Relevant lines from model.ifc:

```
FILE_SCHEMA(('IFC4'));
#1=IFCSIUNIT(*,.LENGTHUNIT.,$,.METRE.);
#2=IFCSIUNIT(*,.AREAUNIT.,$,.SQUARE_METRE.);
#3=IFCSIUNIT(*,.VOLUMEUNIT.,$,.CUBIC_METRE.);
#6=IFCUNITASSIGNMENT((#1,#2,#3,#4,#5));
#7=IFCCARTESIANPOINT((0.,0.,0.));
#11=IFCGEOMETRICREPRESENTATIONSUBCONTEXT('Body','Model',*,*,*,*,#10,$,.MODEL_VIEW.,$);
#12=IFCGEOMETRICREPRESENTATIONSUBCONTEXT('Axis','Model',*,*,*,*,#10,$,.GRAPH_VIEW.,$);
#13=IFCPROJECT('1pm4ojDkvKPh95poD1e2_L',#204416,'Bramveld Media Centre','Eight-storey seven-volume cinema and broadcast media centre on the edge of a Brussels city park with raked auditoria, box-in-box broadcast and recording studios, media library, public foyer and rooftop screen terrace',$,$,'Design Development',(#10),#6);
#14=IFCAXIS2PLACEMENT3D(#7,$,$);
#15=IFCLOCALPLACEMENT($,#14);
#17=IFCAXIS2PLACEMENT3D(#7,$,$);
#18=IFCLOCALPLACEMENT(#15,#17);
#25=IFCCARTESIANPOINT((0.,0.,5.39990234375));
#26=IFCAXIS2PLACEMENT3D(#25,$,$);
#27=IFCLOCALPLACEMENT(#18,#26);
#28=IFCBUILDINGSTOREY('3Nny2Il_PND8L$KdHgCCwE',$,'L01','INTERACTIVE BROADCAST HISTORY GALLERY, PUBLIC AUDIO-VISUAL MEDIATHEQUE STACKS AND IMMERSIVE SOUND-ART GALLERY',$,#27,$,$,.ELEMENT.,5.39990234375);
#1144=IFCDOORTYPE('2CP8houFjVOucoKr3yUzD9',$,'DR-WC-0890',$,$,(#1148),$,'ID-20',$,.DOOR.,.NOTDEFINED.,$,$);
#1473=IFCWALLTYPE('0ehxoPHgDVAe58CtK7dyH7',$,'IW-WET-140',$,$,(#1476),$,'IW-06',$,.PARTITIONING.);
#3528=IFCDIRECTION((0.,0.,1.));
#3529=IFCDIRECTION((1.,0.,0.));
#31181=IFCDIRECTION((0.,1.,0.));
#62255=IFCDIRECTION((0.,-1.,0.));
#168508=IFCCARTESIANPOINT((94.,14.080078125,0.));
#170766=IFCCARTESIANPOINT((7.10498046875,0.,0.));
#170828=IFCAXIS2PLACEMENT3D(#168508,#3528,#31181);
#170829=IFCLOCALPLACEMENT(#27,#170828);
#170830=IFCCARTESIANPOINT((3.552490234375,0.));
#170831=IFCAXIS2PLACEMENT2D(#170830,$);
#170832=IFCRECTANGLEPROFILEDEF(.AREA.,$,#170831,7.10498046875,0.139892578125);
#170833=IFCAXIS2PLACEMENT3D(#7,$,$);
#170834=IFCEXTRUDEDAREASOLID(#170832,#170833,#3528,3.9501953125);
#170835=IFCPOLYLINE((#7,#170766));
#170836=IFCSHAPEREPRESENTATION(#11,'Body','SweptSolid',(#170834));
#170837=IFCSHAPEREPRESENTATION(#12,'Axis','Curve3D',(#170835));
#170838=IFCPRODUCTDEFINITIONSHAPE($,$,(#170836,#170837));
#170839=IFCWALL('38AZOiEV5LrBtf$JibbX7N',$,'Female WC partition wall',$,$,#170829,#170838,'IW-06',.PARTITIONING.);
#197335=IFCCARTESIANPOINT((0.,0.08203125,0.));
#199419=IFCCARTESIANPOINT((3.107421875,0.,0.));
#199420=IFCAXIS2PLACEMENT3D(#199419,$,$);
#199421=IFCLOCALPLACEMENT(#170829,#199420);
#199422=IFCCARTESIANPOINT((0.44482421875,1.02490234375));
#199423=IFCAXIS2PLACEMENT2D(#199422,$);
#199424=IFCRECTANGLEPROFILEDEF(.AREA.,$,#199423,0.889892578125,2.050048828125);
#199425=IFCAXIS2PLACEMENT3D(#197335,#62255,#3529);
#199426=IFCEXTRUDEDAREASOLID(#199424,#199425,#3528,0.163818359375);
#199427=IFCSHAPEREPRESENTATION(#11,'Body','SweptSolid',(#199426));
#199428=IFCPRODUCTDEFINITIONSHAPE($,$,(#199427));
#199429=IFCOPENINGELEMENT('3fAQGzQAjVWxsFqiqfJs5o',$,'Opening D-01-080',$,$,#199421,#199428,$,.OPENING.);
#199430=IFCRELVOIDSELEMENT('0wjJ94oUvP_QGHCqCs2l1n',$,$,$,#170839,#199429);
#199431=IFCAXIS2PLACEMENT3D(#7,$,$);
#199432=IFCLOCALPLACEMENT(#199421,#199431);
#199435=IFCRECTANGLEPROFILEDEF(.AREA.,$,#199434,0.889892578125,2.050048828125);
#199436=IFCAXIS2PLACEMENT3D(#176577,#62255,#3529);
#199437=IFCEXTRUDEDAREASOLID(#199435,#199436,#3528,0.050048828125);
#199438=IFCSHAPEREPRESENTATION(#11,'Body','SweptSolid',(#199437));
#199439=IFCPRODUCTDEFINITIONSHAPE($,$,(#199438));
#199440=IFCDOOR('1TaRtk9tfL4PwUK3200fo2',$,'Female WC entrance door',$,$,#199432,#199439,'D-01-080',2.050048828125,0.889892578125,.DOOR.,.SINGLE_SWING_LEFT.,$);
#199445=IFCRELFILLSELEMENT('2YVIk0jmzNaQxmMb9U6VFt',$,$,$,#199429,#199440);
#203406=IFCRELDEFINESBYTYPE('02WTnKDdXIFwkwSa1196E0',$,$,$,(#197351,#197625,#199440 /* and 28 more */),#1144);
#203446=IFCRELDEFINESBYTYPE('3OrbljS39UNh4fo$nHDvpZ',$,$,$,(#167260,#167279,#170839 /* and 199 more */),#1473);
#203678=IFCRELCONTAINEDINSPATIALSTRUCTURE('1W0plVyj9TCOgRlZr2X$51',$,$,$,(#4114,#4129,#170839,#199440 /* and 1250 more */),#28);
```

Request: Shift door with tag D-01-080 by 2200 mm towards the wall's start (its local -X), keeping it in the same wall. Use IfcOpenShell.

```python
import ifcopenshell
import ifcopenshell.api.geometry
import ifcopenshell.util.placement

model = ifcopenshell.open("model.ifc")

door = model.by_guid("1TaRtk9tfL4PwUK3200fo2")
opening = door.FillsVoids[0].RelatingOpeningElement
wall = opening.VoidsElements[0].RelatingBuildingElement

wall_matrix = ifcopenshell.util.placement.get_local_placement(wall.ObjectPlacement)
shift = wall_matrix[:3, 0] * -2.2
before = ifcopenshell.util.placement.get_local_placement(door.ObjectPlacement)[:3, 3].copy()

# The door is placed relative to its opening, so it follows when the opening moves.
matrix = ifcopenshell.util.placement.get_local_placement(opening.ObjectPlacement)
matrix[:3, 3] += shift
ifcopenshell.api.geometry.edit_object_placement(
    model, product=opening, matrix=matrix, is_si=False, should_transform_children=True
)

after = ifcopenshell.util.placement.get_local_placement(door.ObjectPlacement)[:3, 3]
print("door moved by", (after - before).round(3) + 0.0)

model.write("model_updated.ifc")
```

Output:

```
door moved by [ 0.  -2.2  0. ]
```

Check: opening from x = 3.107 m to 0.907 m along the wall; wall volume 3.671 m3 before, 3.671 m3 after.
